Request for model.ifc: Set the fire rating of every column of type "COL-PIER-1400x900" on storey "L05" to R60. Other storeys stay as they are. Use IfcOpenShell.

First a look at what the model holds.

```python
import ifcopenshell
import ifcopenshell.util.element

model = ifcopenshell.open("model.ifc")
print(model.schema)
storey = next(s for s in model.by_type("IfcBuildingStorey") if s.Name == "L05")
columns = [e for e in ifcopenshell.util.element.get_decomposition(storey) if e.is_a("IfcColumn")]
seen = {}
for e in columns:
    element_type = ifcopenshell.util.element.get_type(e)
    key = (element_type.Name if element_type != e and element_type else None, ifcopenshell.util.element.get_pset(e, "Pset_ColumnCommon", "FireRating"))
    seen[key] = seen.get(key, 0) + 1
for (name, value), count in sorted(seen.items(), key=str):
    print(count, "x", name, "|", value)
```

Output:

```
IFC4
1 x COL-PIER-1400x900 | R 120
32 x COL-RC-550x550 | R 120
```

```python
import ifcopenshell
import ifcopenshell.api.pset
import ifcopenshell.util.element

model = ifcopenshell.open("model.ifc")

storey = next(s for s in model.by_type("IfcBuildingStorey") if s.Name == "L05")
columns = [e for e in ifcopenshell.util.element.get_decomposition(storey) if e.is_a("IfcColumn")]

count = 0
for e in columns:
    element_type = ifcopenshell.util.element.get_type(e)
    if element_type in (None, e) or element_type.Name != "COL-PIER-1400x900":
        continue
    # add_pset returns the element's existing set when there is one.
    pset = ifcopenshell.api.pset.add_pset(model, product=e, name="Pset_ColumnCommon")
    ifcopenshell.api.pset.edit_pset(model, pset=pset, properties={"FireRating": "R60"})
    count += 1

print(count, "columns updated")

model.write("model_updated.ifc")
```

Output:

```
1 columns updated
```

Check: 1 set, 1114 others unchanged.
